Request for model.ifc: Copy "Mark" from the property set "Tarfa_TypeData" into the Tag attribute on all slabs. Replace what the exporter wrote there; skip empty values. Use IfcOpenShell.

First a look at what the model holds.

```python
import ifcopenshell
import ifcopenshell.util.element

model = ifcopenshell.open("model.ifc")
print(model.schema)
slabs = model.by_type("IfcSlab")
print(len(slabs), "slabs")
for e in slabs[:8]:
    source = ifcopenshell.util.element.get_pset(e, "Tarfa_TypeData", "Mark")
    target = e.Tag
    print(e.id(), repr(source), repr(target), sep=" | ")
```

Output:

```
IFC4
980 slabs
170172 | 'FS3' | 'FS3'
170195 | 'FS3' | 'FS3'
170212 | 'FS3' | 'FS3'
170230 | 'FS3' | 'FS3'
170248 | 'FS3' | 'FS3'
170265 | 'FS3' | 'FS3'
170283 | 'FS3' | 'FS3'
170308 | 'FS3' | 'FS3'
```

```python
import ifcopenshell
import ifcopenshell.util.element

model = ifcopenshell.open("model.ifc")

count = 0
for e in model.by_type("IfcSlab"):
    value = ifcopenshell.util.element.get_pset(e, "Tarfa_TypeData", "Mark")
    current = e.Tag
    if not value or not value.strip() or current == value:
        continue
    e.Tag = value
    count += 1

print(count, "slabs updated")

model.write("model-out.ifc")
```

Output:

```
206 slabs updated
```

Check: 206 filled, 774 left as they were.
